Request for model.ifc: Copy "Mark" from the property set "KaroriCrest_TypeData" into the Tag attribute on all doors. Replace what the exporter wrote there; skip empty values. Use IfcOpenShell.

First a look at what the model holds.

```python
import ifcopenshell
import ifcopenshell.util.element

model = ifcopenshell.open("model.ifc")
print(model.schema)
doors = model.by_type("IfcDoor")
print(len(doors), "doors")
for e in doors[:8]:
    source = ifcopenshell.util.element.get_pset(e, "KaroriCrest_TypeData", "Mark")
    target = e.Tag
    print(e.id(), repr(source), repr(target), sep=" | ")
```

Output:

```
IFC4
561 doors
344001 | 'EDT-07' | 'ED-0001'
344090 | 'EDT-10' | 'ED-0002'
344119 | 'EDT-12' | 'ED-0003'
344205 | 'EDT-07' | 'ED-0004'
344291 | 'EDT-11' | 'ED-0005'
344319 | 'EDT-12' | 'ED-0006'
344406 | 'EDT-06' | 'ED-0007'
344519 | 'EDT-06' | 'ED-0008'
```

```python
import ifcopenshell
import ifcopenshell.util.element

model = ifcopenshell.open("model.ifc")

count = 0
for e in model.by_type("IfcDoor"):
    value = ifcopenshell.util.element.get_pset(e, "KaroriCrest_TypeData", "Mark")
    current = e.Tag
    if not value or not value.strip() or current == value:
        continue
    e.Tag = value
    count += 1

print(count, "doors updated")

model.write("model_v2.ifc")
```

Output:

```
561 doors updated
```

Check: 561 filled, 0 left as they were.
